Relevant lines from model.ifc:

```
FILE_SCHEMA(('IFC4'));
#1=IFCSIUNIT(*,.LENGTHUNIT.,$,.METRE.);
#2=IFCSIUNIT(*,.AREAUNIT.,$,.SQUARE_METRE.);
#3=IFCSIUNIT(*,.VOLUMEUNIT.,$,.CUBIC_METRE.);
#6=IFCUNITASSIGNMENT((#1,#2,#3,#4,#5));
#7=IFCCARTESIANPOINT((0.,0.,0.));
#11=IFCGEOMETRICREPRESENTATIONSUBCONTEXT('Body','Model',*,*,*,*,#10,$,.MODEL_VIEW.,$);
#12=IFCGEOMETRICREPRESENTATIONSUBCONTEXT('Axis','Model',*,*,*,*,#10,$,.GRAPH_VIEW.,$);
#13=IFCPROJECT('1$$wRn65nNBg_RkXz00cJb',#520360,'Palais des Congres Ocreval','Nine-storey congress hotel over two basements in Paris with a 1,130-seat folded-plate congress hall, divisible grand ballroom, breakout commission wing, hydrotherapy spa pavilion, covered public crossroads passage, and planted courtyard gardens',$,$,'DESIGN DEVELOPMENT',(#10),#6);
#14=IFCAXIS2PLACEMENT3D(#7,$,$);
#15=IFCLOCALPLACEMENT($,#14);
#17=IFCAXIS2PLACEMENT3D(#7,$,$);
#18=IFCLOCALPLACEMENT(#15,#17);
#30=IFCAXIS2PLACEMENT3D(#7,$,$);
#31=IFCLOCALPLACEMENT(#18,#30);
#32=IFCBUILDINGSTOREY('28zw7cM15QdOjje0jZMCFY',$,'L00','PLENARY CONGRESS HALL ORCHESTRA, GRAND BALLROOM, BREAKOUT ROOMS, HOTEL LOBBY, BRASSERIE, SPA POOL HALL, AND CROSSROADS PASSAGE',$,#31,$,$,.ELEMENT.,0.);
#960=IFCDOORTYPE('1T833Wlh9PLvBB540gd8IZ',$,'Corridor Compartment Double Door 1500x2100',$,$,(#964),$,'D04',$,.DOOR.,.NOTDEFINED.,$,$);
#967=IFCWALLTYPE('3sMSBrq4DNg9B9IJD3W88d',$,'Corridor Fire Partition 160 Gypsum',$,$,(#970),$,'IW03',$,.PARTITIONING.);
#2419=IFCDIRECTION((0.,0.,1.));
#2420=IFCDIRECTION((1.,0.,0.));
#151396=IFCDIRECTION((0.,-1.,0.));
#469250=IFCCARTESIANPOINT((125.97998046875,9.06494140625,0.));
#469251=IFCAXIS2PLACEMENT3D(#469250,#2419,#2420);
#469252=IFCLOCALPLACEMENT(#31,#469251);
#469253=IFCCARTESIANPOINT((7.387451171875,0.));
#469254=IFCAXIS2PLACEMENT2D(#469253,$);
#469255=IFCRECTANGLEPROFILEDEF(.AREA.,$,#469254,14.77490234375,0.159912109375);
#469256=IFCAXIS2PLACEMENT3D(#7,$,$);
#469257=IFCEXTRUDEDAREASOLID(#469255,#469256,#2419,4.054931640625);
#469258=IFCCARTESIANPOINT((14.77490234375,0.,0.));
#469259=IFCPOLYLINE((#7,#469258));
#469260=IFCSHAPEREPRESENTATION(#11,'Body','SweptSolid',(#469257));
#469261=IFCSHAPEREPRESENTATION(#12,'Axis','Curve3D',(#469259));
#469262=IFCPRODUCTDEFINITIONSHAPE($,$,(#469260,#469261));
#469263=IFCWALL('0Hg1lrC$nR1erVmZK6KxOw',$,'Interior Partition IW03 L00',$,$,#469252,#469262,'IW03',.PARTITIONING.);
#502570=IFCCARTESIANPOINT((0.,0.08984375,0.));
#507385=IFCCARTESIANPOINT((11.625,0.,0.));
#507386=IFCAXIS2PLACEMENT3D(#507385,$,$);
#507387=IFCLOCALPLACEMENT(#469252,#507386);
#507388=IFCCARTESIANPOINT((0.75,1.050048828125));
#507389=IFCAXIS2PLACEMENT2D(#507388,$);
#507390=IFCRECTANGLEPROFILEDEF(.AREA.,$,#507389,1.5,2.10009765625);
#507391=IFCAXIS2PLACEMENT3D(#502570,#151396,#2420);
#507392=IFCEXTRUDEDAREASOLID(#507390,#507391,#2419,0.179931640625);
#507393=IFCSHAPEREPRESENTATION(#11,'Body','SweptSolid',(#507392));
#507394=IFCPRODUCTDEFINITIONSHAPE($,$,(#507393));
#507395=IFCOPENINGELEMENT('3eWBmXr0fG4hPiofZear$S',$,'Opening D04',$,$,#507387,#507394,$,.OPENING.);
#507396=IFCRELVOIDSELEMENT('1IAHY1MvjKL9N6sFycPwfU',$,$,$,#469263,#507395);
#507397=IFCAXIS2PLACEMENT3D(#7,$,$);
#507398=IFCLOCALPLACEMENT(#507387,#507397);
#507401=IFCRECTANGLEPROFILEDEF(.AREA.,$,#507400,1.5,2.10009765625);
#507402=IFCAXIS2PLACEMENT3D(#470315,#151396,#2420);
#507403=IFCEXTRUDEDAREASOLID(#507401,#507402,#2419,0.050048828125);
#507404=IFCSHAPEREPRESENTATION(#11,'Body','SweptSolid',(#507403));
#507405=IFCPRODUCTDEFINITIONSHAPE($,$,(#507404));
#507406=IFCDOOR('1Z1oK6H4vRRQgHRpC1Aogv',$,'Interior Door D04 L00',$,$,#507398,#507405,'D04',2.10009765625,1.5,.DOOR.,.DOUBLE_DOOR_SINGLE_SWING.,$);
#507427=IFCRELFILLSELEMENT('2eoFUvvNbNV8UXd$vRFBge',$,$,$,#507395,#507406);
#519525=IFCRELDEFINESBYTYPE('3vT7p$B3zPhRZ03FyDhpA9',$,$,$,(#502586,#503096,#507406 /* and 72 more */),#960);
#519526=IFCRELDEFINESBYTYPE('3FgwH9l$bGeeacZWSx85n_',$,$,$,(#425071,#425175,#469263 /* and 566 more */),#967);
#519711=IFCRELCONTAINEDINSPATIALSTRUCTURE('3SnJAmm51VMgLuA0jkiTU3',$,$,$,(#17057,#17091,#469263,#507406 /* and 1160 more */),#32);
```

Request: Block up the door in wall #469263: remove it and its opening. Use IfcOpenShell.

```python
import ifcopenshell
import ifcopenshell.api.feature
import ifcopenshell.api.root
import ifcopenshell.geom
import ifcopenshell.util.shape

model = ifcopenshell.open("model.ifc")
settings = ifcopenshell.geom.settings()


def volume(element):
    """Net volume in cubic metres, openings subtracted."""
    shape = ifcopenshell.geom.create_shape(settings, element)
    return ifcopenshell.util.shape.get_volume(shape.geometry)


door = model.by_id(507406)
opening = door.FillsVoids[0].RelatingOpeningElement
wall = opening.VoidsElements[0].RelatingBuildingElement
before = volume(wall)

ifcopenshell.api.root.remove_product(model, product=door)
ifcopenshell.api.feature.remove_feature(model, feature=opening)

after = volume(wall)

print(f"wall volume {before:.3f} -> {after:.3f} m3")

model.write("model_v2.ifc")
```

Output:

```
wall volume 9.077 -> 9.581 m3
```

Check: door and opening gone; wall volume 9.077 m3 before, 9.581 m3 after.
